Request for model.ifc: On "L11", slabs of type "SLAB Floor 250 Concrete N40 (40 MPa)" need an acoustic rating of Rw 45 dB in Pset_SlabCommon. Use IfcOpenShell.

First a look at what the model holds.

```python
import ifcopenshell
import ifcopenshell.util.element

model = ifcopenshell.open("model.ifc")
print(model.schema)
storey = next(s for s in model.by_type("IfcBuildingStorey") if s.Name == "L11")
slabs = [e for e in ifcopenshell.util.element.get_decomposition(storey) if e.is_a("IfcSlab")]
seen = {}
for e in slabs:
    element_type = ifcopenshell.util.element.get_type(e)
    key = (element_type.Name if element_type != e and element_type else None, ifcopenshell.util.element.get_pset(e, "Pset_SlabCommon", "AcousticRating"))
    seen[key] = seen.get(key, 0) + 1
for (name, value), count in sorted(seen.items(), key=str):
    print(count, "x", name, "|", value)
```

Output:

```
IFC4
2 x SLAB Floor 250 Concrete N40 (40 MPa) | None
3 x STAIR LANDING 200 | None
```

```python
import ifcopenshell
import ifcopenshell.api.pset
import ifcopenshell.util.element

model = ifcopenshell.open("model.ifc")

storey = next(s for s in model.by_type("IfcBuildingStorey") if s.Name == "L11")
slabs = [e for e in ifcopenshell.util.element.get_decomposition(storey) if e.is_a("IfcSlab")]

count = 0
for e in slabs:
    element_type = ifcopenshell.util.element.get_type(e)
    if element_type in (None, e) or element_type.Name != "SLAB Floor 250 Concrete N40 (40 MPa)":
        continue
    # add_pset returns the element's existing set when there is one.
    pset = ifcopenshell.api.pset.add_pset(model, product=e, name="Pset_SlabCommon")
    ifcopenshell.api.pset.edit_pset(model, pset=pset, properties={"AcousticRating": "Rw 45 dB"})
    count += 1

print(count, "slabs updated")

model.write("model-out.ifc")
```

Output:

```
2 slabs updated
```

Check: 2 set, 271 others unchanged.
